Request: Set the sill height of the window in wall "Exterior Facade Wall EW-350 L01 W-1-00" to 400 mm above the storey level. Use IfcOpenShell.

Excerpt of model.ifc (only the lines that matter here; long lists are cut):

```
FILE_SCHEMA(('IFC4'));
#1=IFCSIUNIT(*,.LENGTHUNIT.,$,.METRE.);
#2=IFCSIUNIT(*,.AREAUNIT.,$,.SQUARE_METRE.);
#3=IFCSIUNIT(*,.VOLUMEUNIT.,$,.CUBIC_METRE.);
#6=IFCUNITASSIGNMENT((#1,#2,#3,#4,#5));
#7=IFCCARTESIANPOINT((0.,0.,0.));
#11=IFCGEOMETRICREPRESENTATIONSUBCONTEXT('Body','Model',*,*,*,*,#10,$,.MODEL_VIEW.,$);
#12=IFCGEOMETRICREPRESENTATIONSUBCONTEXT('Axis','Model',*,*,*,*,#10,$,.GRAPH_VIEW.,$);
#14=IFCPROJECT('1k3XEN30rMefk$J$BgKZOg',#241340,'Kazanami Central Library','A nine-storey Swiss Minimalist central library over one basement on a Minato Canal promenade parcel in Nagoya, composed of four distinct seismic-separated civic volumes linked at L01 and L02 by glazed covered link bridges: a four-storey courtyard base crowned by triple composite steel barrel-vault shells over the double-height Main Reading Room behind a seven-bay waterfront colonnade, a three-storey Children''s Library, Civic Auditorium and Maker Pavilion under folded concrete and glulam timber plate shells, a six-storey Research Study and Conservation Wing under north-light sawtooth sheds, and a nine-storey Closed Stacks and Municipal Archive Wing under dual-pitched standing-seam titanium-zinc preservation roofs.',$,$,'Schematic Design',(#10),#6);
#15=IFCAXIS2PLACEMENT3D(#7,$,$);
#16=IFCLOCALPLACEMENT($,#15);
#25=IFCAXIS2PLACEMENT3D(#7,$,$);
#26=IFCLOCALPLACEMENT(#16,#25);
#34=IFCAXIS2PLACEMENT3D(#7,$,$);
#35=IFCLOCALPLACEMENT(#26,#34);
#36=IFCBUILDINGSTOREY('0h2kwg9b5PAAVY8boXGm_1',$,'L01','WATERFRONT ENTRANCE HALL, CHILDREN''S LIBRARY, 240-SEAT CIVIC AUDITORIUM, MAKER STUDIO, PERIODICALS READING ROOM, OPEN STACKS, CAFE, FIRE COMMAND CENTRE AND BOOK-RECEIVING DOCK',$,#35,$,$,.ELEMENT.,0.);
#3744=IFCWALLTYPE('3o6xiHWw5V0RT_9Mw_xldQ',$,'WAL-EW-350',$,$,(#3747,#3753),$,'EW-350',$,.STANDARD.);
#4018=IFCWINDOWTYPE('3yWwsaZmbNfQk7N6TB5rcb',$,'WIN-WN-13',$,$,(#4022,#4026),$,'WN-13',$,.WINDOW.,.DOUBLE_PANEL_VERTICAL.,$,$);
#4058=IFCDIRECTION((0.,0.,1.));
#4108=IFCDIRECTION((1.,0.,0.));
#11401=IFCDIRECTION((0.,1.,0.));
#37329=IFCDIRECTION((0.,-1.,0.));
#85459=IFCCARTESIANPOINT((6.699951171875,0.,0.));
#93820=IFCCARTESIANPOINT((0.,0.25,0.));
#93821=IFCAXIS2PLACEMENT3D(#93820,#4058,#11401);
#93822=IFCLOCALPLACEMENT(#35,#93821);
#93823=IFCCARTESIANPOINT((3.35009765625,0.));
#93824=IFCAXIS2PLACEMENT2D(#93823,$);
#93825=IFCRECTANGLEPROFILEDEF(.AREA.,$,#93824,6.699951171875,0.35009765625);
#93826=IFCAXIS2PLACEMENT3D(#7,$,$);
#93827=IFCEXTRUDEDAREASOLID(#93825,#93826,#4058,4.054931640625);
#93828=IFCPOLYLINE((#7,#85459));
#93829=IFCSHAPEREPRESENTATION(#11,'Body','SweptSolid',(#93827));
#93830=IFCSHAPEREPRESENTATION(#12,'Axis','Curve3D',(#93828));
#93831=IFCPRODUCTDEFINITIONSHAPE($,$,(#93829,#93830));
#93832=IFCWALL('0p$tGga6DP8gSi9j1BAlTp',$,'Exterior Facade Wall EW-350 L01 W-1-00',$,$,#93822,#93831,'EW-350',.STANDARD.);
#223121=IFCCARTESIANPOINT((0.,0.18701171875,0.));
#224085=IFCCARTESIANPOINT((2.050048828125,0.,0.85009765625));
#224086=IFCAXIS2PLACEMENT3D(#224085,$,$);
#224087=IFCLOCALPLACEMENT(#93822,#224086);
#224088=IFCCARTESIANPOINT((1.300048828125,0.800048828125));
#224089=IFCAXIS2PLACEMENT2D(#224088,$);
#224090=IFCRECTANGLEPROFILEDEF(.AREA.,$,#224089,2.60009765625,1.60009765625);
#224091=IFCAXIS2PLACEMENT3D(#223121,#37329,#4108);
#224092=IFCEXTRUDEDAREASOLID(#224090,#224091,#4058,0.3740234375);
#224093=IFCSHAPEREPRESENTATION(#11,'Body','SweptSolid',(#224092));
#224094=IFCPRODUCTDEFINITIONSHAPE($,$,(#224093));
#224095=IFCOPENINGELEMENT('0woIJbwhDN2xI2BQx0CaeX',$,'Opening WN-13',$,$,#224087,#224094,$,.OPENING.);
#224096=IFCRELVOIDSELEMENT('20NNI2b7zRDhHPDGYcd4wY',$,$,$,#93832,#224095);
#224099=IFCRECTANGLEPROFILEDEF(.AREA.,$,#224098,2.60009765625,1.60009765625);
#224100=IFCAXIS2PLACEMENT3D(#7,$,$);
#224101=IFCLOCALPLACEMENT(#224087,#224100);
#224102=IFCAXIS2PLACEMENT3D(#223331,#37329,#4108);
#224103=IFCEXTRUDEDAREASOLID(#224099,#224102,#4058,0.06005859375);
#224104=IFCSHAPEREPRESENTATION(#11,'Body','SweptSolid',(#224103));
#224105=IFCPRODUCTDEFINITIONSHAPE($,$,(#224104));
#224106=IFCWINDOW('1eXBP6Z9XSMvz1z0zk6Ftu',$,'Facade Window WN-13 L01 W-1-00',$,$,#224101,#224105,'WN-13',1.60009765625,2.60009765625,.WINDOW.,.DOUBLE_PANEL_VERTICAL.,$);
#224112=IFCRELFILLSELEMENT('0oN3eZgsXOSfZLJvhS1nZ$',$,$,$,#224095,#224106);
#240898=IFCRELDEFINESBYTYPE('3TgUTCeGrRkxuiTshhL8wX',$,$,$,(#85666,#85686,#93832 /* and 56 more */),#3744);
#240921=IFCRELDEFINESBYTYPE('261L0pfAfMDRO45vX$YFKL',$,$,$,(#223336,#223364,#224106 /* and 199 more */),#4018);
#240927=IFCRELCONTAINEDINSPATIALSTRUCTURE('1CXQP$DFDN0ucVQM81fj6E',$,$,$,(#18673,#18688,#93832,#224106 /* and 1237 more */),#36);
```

```python
import numpy as np
import ifcopenshell
import ifcopenshell.api.geometry
import ifcopenshell.geom
import ifcopenshell.util.element
import ifcopenshell.util.placement
import ifcopenshell.util.shape
import ifcopenshell.util.unit

model = ifcopenshell.open("model.ifc")
unit_scale = ifcopenshell.util.unit.calculate_unit_scale(model)

window = model.by_guid("1eXBP6Z9XSMvz1z0zk6Ftu")
opening = window.FillsVoids[0].RelatingOpeningElement
storey = ifcopenshell.util.element.get_container(window, ifc_class="IfcBuildingStorey")
level = ifcopenshell.util.placement.get_local_placement(storey.ObjectPlacement)[2, 3]

# The opening's origin need not be at the sill, so measure its lowest point.
shape = ifcopenshell.geom.create_shape(ifcopenshell.geom.settings(), opening)
bottom = ifcopenshell.util.shape.get_shape_bottom_elevation(shape, shape.geometry) / unit_scale
dz = level + 0.4 - bottom

shift = np.array([0.0, 0.0, dz])
# The window is placed relative to its opening, so it follows when the opening moves.
matrix = ifcopenshell.util.placement.get_local_placement(opening.ObjectPlacement)
matrix[:3, 3] += shift
ifcopenshell.api.geometry.edit_object_placement(
    model, product=opening, matrix=matrix, is_si=False, should_transform_children=True
)

print(f"moved by {dz * unit_scale:+.3f} m")

model.write("model_v2.ifc")
```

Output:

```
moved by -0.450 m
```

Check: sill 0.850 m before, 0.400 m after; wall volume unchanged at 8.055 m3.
